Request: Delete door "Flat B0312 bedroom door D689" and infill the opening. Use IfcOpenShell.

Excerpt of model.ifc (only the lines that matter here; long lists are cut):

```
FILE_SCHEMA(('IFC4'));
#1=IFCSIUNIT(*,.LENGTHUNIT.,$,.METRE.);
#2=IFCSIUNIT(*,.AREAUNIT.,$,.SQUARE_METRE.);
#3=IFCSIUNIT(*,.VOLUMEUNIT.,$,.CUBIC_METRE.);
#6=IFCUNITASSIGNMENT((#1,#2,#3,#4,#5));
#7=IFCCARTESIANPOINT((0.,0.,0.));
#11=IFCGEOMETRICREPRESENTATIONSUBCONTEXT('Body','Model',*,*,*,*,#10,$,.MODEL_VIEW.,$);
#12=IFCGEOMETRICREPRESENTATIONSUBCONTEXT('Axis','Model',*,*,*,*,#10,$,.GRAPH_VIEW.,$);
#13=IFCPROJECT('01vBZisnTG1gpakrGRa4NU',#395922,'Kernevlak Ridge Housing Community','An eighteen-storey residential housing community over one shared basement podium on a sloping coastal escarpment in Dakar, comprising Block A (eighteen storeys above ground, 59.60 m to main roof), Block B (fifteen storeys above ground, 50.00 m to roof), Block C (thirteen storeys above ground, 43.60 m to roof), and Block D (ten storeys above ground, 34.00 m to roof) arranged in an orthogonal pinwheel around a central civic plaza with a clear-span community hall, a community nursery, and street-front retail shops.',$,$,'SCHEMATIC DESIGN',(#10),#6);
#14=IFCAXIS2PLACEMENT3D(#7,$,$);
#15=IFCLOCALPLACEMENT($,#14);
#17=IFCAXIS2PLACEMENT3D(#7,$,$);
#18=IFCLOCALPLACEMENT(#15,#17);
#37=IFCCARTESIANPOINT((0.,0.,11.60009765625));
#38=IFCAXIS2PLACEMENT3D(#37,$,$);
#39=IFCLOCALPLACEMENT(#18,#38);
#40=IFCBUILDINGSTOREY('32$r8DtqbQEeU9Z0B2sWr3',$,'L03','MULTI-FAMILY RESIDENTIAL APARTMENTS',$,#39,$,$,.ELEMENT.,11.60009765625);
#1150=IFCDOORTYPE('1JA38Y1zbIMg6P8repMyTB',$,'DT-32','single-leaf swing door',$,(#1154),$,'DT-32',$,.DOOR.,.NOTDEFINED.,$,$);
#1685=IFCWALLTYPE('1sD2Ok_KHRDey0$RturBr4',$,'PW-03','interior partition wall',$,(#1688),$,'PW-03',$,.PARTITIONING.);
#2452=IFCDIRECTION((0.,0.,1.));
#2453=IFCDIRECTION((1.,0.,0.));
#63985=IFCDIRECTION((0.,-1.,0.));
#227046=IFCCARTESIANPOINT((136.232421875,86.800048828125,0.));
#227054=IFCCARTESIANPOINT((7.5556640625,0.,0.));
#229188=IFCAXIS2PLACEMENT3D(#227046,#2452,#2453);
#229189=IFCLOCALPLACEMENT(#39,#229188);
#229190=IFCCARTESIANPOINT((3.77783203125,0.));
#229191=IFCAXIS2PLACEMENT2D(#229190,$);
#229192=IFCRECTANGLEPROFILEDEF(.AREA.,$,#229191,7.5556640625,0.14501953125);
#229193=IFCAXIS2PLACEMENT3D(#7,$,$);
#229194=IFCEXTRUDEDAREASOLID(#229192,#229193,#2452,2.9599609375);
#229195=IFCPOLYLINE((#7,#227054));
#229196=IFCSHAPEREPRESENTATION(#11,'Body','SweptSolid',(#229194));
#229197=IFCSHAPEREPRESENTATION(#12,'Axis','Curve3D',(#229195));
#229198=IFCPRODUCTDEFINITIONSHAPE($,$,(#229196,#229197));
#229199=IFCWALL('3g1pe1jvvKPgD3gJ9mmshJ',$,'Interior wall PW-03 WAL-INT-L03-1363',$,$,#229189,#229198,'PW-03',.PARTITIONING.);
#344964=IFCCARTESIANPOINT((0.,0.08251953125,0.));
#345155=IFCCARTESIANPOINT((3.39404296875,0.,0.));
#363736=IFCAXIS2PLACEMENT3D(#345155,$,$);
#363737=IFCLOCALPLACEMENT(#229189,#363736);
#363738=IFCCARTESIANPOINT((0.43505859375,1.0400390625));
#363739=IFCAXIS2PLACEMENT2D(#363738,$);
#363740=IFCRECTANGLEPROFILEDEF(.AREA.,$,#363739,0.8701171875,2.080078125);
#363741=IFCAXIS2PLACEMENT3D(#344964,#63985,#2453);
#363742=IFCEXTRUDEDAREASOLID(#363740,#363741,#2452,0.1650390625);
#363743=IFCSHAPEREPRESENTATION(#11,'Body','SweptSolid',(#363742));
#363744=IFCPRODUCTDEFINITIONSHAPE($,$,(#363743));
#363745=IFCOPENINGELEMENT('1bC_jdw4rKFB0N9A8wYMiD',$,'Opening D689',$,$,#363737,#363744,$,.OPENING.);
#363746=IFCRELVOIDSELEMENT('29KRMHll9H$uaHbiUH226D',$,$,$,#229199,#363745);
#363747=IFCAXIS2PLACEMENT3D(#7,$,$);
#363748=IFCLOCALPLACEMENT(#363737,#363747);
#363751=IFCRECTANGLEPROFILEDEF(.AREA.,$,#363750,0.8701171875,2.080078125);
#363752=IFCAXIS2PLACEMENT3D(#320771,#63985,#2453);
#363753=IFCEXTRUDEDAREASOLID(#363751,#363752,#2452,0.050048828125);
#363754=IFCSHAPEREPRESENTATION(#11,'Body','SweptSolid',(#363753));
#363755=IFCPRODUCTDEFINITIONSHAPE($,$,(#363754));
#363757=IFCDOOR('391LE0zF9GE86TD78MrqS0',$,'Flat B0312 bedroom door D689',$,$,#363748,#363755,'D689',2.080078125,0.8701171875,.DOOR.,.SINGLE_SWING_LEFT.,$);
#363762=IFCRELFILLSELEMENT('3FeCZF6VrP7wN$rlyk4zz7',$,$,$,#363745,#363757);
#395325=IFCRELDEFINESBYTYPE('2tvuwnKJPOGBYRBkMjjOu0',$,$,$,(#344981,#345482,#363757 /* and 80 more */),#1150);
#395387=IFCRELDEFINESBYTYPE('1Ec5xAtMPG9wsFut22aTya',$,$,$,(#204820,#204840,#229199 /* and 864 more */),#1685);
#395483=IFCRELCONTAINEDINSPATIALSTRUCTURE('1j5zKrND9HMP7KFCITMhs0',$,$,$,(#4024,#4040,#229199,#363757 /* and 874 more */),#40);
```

```python
import ifcopenshell
import ifcopenshell.api.feature
import ifcopenshell.api.root
import ifcopenshell.geom
import ifcopenshell.util.shape

model = ifcopenshell.open("model.ifc")
settings = ifcopenshell.geom.settings()


def volume(element):
    """Net volume in cubic metres, openings subtracted."""
    shape = ifcopenshell.geom.create_shape(settings, element)
    return ifcopenshell.util.shape.get_volume(shape.geometry)


door = model.by_guid("391LE0zF9GE86TD78MrqS0")
opening = door.FillsVoids[0].RelatingOpeningElement
wall = opening.VoidsElements[0].RelatingBuildingElement
before = volume(wall)

ifcopenshell.api.root.remove_product(model, product=door)
ifcopenshell.api.feature.remove_feature(model, feature=opening)

after = volume(wall)

print(f"wall volume {before:.3f} -> {after:.3f} m3")

model.write("model_v2.ifc")
```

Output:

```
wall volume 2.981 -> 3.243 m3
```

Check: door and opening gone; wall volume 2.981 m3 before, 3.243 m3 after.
